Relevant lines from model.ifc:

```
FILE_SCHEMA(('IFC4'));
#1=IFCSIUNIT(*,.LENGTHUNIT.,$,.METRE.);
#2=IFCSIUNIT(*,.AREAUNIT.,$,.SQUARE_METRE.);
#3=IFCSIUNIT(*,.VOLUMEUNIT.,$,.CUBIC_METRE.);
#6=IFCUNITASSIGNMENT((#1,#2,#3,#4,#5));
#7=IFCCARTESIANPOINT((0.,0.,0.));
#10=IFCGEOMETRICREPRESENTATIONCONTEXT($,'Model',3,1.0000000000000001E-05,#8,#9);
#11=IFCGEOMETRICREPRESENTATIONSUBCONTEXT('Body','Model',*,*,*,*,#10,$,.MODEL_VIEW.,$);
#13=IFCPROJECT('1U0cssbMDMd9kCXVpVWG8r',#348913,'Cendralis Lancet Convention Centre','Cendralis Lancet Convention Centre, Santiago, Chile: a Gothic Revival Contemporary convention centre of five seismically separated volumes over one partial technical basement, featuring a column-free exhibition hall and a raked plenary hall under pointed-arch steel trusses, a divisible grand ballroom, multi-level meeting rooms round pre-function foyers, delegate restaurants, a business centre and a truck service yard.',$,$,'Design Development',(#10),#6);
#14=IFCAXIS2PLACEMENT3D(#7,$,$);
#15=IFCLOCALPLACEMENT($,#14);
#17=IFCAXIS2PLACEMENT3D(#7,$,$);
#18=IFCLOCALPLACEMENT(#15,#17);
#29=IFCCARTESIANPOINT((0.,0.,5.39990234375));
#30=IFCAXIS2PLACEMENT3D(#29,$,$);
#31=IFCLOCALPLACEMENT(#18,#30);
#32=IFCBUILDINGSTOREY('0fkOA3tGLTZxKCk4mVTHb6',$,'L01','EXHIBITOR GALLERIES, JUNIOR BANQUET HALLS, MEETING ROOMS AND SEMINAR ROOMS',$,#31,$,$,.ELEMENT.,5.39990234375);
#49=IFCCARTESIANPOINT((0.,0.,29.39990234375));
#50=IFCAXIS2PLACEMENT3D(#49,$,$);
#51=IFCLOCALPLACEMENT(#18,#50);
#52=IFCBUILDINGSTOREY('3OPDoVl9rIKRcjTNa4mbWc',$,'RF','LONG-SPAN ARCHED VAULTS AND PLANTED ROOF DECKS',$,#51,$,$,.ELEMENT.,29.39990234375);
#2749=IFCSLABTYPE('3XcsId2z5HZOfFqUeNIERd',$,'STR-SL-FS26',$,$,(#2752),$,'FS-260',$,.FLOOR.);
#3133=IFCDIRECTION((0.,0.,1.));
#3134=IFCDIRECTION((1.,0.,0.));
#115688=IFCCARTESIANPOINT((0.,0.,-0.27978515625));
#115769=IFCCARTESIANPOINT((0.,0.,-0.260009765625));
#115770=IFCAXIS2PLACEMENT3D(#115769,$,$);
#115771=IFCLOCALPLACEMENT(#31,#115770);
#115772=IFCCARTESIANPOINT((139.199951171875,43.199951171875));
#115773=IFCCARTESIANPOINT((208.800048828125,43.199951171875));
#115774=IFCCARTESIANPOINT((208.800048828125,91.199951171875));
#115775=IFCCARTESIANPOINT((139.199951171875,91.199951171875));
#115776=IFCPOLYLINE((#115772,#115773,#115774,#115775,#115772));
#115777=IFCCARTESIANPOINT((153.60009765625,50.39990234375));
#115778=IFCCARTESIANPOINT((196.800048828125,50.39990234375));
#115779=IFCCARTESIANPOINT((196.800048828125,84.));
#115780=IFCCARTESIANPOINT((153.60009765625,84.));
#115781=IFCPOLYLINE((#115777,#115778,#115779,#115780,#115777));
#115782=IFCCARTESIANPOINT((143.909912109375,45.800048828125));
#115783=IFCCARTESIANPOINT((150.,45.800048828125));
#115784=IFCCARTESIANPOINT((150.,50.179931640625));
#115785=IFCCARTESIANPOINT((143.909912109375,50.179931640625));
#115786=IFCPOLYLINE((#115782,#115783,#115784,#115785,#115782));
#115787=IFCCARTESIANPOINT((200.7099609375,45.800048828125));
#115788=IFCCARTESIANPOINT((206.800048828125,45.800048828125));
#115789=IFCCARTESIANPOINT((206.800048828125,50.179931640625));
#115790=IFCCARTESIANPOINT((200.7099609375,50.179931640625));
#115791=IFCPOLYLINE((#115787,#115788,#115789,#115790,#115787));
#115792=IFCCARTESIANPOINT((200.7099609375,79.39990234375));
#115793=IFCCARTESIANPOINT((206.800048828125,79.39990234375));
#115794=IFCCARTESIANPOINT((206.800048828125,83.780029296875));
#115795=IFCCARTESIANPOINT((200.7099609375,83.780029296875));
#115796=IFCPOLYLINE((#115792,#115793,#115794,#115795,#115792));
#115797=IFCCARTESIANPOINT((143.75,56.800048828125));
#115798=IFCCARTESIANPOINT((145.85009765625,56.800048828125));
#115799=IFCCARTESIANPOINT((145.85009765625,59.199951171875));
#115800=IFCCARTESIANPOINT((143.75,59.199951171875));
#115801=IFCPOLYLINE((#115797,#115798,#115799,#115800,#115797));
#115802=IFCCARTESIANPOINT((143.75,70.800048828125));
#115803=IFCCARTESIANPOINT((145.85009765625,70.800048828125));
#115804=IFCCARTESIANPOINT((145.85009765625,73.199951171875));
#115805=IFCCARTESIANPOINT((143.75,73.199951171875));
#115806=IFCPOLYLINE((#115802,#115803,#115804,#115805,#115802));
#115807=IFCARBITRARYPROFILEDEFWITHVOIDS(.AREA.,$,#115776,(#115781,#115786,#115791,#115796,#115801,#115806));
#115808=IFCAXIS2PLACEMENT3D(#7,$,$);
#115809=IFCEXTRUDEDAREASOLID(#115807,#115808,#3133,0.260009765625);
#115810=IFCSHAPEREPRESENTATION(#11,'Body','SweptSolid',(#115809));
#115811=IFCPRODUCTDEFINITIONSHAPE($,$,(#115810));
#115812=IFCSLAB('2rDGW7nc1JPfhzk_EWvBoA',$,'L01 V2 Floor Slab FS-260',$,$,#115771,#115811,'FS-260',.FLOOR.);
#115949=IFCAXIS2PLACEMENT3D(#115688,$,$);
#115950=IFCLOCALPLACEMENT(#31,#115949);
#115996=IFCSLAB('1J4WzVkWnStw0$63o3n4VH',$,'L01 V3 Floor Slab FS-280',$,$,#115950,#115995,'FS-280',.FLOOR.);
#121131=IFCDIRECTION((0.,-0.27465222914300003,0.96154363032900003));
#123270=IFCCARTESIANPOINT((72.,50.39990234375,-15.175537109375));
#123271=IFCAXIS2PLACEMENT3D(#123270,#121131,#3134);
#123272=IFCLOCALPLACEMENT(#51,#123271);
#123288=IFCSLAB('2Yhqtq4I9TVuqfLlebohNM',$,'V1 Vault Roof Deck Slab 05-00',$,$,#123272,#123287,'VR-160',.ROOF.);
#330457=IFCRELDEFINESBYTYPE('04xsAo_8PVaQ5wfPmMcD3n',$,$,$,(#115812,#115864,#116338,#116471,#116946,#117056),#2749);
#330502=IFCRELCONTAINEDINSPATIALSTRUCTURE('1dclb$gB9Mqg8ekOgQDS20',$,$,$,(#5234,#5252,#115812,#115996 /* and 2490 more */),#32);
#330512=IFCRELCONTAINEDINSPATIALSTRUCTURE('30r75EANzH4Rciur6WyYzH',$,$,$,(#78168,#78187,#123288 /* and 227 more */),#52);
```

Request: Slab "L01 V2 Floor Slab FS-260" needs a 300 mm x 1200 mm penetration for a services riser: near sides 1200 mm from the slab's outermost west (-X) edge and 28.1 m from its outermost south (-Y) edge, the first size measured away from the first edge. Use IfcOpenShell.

```python
import numpy as np
import ifcopenshell
import ifcopenshell.api.feature
import ifcopenshell.api.geometry
import ifcopenshell.api.root
import ifcopenshell.geom
import ifcopenshell.util.placement
import ifcopenshell.util.representation
import ifcopenshell.util.shape
import ifcopenshell.util.unit

model = ifcopenshell.open("model.ifc")
unit_scale = ifcopenshell.util.unit.calculate_unit_scale(model)
settings = ifcopenshell.geom.settings()


def volume(element):
    """Net volume in cubic metres, openings subtracted."""
    shape = ifcopenshell.geom.create_shape(settings, element)
    return ifcopenshell.util.shape.get_volume(shape.geometry)


slab = model.by_guid("2rDGW7nc1JPfhzk_EWvBoA")
before = volume(slab)

# Extent in the slab's own axes, in metres. The edges named are its -X and -Y sides.
slab_shape = ifcopenshell.geom.create_shape(settings, slab)
vertices = ifcopenshell.util.shape.get_vertices(slab_shape.geometry)
x_min, y_min, bottom = vertices.min(axis=0)
top = vertices[:, 2].max()

opening = ifcopenshell.api.root.create_entity(model, ifc_class="IfcOpeningElement", name="Services riser opening", predefined_type="OPENING")
context = ifcopenshell.util.representation.get_context(model, "Model", "Body", "MODEL_VIEW")
width, depth = 0.3, 1.2
outline = [(0.0, 0.0), (width, 0.0), (width, depth), (0.0, depth), (0.0, 0.0)]
# Overshoot both faces by 50 mm so the cut is clean.
shape = ifcopenshell.api.geometry.add_slab_representation(
    model, context=context, depth=top - bottom + 0.1, polyline=outline
)
ifcopenshell.api.geometry.assign_representation(model, product=opening, representation=shape)

matrix = ifcopenshell.util.placement.get_local_placement(slab.ObjectPlacement)
matrix[:, 3] = matrix @ np.append(np.array([x_min + 1.2, y_min + 28.1, bottom - 0.05]) / unit_scale, 1.0)
ifcopenshell.api.geometry.edit_object_placement(model, product=opening, matrix=matrix, is_si=False)
ifcopenshell.api.feature.add_feature(model, feature=opening, element=slab)

after = volume(slab)

print(f"slab volume {before:.3f} -> {after:.3f} m3")

model.write("model_rev.ifc")
```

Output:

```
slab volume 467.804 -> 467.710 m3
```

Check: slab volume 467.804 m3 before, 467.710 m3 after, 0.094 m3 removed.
